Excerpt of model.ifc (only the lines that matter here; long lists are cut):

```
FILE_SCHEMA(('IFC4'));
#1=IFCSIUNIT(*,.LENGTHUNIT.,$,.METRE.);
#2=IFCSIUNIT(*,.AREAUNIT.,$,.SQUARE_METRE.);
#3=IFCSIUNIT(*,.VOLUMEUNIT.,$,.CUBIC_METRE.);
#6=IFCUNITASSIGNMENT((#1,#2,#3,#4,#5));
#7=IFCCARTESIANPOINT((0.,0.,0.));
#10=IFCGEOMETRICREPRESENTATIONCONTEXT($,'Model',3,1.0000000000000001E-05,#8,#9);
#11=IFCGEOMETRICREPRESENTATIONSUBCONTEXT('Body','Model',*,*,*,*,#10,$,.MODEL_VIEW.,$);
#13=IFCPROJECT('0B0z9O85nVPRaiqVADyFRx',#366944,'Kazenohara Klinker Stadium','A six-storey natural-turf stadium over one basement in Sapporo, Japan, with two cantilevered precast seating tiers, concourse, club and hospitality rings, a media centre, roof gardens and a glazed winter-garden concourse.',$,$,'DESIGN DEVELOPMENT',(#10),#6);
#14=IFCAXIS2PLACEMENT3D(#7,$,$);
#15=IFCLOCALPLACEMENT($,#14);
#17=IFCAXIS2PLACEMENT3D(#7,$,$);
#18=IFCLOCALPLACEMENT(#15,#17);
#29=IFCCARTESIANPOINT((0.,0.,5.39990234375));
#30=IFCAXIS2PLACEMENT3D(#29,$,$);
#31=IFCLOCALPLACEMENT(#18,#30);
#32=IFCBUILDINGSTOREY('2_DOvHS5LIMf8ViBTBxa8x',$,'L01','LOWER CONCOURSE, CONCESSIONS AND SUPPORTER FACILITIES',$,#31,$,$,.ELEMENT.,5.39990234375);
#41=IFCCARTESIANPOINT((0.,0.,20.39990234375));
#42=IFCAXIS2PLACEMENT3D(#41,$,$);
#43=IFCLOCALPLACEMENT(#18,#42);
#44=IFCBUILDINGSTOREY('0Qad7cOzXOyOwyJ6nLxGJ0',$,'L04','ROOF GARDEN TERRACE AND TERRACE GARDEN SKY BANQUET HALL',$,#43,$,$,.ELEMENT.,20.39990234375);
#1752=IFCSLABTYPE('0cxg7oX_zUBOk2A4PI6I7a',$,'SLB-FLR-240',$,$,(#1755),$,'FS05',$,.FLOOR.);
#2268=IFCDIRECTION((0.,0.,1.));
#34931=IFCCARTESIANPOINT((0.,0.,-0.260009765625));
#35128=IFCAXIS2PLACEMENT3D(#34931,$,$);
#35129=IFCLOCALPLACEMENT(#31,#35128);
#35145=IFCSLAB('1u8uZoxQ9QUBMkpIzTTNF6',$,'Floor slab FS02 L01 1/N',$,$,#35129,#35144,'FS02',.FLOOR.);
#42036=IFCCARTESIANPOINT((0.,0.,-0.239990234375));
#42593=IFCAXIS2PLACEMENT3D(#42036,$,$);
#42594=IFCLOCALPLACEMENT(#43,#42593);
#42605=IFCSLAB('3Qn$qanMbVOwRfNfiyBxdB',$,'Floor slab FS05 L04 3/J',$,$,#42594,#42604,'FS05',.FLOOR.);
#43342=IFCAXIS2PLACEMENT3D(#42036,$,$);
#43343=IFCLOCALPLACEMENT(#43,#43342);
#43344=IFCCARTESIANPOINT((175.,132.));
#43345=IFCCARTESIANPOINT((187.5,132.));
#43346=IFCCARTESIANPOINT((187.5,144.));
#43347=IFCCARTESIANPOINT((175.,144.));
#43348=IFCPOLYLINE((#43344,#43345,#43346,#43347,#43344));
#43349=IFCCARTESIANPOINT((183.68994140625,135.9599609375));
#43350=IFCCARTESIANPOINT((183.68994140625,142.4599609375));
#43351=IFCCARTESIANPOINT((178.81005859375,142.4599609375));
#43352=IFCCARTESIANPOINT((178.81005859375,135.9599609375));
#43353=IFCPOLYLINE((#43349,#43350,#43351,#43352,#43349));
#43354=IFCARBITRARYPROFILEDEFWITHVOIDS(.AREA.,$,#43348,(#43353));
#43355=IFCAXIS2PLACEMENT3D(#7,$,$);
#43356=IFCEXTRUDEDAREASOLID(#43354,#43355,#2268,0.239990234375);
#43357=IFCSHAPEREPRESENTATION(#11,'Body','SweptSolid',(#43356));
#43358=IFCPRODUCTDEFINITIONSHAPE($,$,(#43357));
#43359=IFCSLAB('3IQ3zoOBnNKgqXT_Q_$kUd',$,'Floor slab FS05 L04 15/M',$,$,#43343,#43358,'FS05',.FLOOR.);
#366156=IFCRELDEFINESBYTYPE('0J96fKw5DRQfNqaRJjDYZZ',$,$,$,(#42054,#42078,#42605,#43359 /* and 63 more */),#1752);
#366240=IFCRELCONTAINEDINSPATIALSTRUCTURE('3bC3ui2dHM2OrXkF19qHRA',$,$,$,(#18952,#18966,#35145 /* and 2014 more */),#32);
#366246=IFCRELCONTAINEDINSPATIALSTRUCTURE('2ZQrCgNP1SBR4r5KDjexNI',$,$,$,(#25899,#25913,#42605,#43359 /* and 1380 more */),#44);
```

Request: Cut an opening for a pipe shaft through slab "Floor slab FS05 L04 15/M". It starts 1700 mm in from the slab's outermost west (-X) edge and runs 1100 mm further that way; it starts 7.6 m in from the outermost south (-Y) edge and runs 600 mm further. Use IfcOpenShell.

```python
import numpy as np
import ifcopenshell
import ifcopenshell.api.feature
import ifcopenshell.api.geometry
import ifcopenshell.api.root
import ifcopenshell.geom
import ifcopenshell.util.placement
import ifcopenshell.util.representation
import ifcopenshell.util.shape
import ifcopenshell.util.unit

model = ifcopenshell.open("model.ifc")
unit_scale = ifcopenshell.util.unit.calculate_unit_scale(model)
settings = ifcopenshell.geom.settings()


def volume(element):
    """Net volume in cubic metres, openings subtracted."""
    shape = ifcopenshell.geom.create_shape(settings, element)
    return ifcopenshell.util.shape.get_volume(shape.geometry)


slab = model.by_guid("3IQ3zoOBnNKgqXT_Q_$kUd")
before = volume(slab)

# Extent in the slab's own axes, in metres. The edges named are its -X and -Y sides.
slab_shape = ifcopenshell.geom.create_shape(settings, slab)
vertices = ifcopenshell.util.shape.get_vertices(slab_shape.geometry)
x_min, y_min, bottom = vertices.min(axis=0)
top = vertices[:, 2].max()

opening = ifcopenshell.api.root.create_entity(model, ifc_class="IfcOpeningElement", name="Pipe shaft opening", predefined_type="OPENING")
context = ifcopenshell.util.representation.get_context(model, "Model", "Body", "MODEL_VIEW")
width, depth = 1.1, 0.6
outline = [(0.0, 0.0), (width, 0.0), (width, depth), (0.0, depth), (0.0, 0.0)]
# Overshoot both faces by 50 mm so the cut is clean.
shape = ifcopenshell.api.geometry.add_slab_representation(
    model, context=context, depth=top - bottom + 0.1, polyline=outline
)
ifcopenshell.api.geometry.assign_representation(model, product=opening, representation=shape)

matrix = ifcopenshell.util.placement.get_local_placement(slab.ObjectPlacement)
matrix[:, 3] = matrix @ np.append(np.array([x_min + 1.7, y_min + 7.6, bottom - 0.05]) / unit_scale, 1.0)
ifcopenshell.api.geometry.edit_object_placement(model, product=opening, matrix=matrix, is_si=False)
ifcopenshell.api.feature.add_feature(model, feature=opening, element=slab)

after = volume(slab)

print(f"slab volume {before:.3f} -> {after:.3f} m3")

model.write("model_v2.ifc")
```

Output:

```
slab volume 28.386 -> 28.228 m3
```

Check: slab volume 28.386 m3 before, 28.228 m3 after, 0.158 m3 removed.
